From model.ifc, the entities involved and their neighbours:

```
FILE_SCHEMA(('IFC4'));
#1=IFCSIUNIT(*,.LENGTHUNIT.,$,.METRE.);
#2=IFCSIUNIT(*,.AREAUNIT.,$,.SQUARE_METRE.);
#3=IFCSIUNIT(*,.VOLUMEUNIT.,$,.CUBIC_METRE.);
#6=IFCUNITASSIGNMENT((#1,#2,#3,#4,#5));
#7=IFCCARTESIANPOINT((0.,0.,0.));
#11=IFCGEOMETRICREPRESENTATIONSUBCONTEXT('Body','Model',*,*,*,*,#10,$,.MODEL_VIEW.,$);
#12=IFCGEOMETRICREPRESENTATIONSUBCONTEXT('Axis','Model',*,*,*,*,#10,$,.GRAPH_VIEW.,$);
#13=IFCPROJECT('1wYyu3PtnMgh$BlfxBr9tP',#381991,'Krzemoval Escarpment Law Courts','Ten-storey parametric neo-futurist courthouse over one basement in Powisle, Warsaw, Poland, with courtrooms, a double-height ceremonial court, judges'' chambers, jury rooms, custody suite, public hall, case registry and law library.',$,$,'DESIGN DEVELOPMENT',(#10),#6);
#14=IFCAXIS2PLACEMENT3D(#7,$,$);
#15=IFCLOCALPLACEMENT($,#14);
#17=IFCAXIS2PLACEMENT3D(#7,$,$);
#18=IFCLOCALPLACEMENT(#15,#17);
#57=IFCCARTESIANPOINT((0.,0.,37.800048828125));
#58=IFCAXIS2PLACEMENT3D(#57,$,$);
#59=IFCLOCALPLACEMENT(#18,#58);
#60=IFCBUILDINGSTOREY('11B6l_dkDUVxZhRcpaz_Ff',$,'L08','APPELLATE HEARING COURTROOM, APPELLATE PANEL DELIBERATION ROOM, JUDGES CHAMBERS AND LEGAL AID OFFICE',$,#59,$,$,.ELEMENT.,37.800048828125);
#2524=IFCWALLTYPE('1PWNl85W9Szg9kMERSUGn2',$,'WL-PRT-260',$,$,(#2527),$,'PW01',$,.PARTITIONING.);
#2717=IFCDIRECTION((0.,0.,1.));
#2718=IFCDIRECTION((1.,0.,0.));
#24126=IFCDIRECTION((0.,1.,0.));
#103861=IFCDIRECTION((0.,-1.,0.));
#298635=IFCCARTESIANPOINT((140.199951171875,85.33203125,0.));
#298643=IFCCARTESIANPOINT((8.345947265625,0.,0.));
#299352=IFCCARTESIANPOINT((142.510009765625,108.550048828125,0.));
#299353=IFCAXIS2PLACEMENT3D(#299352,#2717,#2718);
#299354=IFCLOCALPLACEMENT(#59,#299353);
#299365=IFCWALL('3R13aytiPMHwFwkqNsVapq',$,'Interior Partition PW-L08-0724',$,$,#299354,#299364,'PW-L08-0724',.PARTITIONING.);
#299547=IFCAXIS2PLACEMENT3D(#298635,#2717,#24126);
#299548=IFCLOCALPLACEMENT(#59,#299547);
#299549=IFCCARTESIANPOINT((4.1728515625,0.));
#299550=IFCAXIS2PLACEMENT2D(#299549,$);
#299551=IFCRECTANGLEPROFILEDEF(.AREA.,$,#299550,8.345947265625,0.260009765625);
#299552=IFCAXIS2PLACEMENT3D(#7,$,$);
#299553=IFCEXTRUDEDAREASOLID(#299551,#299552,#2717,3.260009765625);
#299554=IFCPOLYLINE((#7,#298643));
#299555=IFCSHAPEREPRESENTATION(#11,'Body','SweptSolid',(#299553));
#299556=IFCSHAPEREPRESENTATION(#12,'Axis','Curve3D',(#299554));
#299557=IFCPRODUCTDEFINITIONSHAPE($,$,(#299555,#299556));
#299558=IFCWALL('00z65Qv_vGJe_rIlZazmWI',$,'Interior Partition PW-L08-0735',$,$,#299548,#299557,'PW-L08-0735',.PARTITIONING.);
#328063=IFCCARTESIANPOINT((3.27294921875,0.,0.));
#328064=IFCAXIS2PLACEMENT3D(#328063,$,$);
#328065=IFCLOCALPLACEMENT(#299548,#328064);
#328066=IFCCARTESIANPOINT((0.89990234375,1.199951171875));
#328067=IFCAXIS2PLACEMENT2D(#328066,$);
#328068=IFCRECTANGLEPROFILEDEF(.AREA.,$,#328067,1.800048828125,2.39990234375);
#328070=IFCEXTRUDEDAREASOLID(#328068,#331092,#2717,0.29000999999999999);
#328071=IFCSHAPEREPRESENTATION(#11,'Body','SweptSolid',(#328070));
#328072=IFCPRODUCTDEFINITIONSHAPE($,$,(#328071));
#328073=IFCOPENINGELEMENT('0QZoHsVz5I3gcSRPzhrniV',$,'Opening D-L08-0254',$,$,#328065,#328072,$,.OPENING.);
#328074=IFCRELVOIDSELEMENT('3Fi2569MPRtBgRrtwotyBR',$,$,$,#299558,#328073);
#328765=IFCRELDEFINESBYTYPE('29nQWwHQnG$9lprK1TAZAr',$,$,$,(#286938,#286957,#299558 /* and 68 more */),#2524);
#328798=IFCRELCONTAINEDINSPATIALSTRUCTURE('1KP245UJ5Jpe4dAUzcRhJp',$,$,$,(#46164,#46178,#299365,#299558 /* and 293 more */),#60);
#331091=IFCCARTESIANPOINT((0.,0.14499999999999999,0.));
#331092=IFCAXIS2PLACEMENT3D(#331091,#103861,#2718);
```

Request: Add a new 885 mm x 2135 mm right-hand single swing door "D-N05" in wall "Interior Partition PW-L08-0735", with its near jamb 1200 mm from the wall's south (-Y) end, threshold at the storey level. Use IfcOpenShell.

```python
import numpy as np
import ifcopenshell
import ifcopenshell.api.feature
import ifcopenshell.api.geometry
import ifcopenshell.api.root
import ifcopenshell.api.spatial
import ifcopenshell.geom
import ifcopenshell.util.element
import ifcopenshell.util.placement
import ifcopenshell.util.representation
import ifcopenshell.util.shape
import ifcopenshell.util.unit

model = ifcopenshell.open("model.ifc")
unit_scale = ifcopenshell.util.unit.calculate_unit_scale(model)
settings = ifcopenshell.geom.settings()


def volume(element):
    """Net volume in cubic metres, openings subtracted."""
    shape = ifcopenshell.geom.create_shape(settings, element)
    return ifcopenshell.util.shape.get_volume(shape.geometry)


wall = model.by_guid("00z65Qv_vGJe_rIlZazmWI")
storey = ifcopenshell.util.element.get_container(wall, ifc_class="IfcBuildingStorey")
context = ifcopenshell.util.representation.get_context(model, "Model", "Body", "MODEL_VIEW")
before = volume(wall)

width, height, from_end, sill = 0.885, 2.135, 1.2, 0.0  # metres

# The wall runs along its own X axis, and the end named is its -X end.
wall_shape = ifcopenshell.geom.create_shape(settings, wall)
x, y, z = ifcopenshell.util.shape.get_vertices(wall_shape.geometry).T
start = x.min() + from_end
face, thickness = float(y.min()), float(y.max() - y.min())
wall_matrix = ifcopenshell.util.placement.get_local_placement(wall.ObjectPlacement)
level = ifcopenshell.util.placement.get_local_placement(storey.ObjectPlacement)[2, 3]


def in_wall(x, y):
    """Placement at x, y metres in the wall's axes, at sill height."""
    matrix = wall_matrix.copy()
    matrix[:, 3] = wall_matrix @ np.array([x / unit_scale, y / unit_scale, 0.0, 1.0])
    matrix[2, 3] = level + sill / unit_scale
    return matrix


# Opening: a box that overshoots both wall faces by 50 mm.
opening = ifcopenshell.api.root.create_entity(model, ifc_class="IfcOpeningElement", predefined_type="OPENING")
box = ifcopenshell.api.geometry.add_wall_representation(
    model, context=context, length=width, height=height, thickness=thickness + 0.1
)
ifcopenshell.api.geometry.assign_representation(model, product=opening, representation=box)
ifcopenshell.api.geometry.edit_object_placement(model, product=opening, matrix=in_wall(start, face - 0.05), is_si=False)
ifcopenshell.api.feature.add_feature(model, feature=opening, element=wall)

door = ifcopenshell.api.root.create_entity(model, ifc_class="IfcDoor", name="D-N05", predefined_type="DOOR")
door.OverallWidth, door.OverallHeight = width / unit_scale, height / unit_scale
door.OperationType = "SINGLE_SWING_RIGHT"
body = ifcopenshell.api.geometry.add_door_representation(
    model,
    context=context,
    overall_width=door.OverallWidth,
    overall_height=door.OverallHeight,
    operation_type="SINGLE_SWING_RIGHT",
    lining_properties={"LiningDepth": thickness / unit_scale, "ThresholdDepth": thickness / unit_scale},
)
ifcopenshell.api.geometry.assign_representation(model, product=door, representation=body)
ifcopenshell.api.spatial.assign_container(model, products=[door], relating_structure=storey)
ifcopenshell.api.feature.add_filling(model, opening=opening, element=door)

# The lining spans the wall, so the door starts at the wall face.
ifcopenshell.api.geometry.edit_object_placement(model, product=door, matrix=in_wall(start, face), is_si=False)

after = volume(wall)

print(f"wall volume {before:.3f} -> {after:.3f} m3")

model.write("model_updated.ifc")
```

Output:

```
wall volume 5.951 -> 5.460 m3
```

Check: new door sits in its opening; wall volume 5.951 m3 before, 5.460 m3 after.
